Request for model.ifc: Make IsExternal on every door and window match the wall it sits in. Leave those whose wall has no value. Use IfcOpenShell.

First a look at what the model holds.

```python
import ifcopenshell
import ifcopenshell.util.element

model = ifcopenshell.open("model.ifc")
print(model.schema)
seen = {}
for e in model.by_type("IfcDoor") + model.by_type("IfcWindow"):
    if not e.FillsVoids:
        continue
    host = e.FillsVoids[0].RelatingOpeningElement.VoidsElements[0].RelatingBuildingElement
    own = ifcopenshell.util.element.get_pset(e, f"Pset_{e.is_a()[3:].removesuffix('StandardCase')}Common", "IsExternal")
    wall = ifcopenshell.util.element.get_pset(host, "Pset_WallCommon", "IsExternal")
    seen[e.is_a(), own, wall] = seen.get((e.is_a(), own, wall), 0) + 1
for (cls, own, wall), count in sorted(seen.items(), key=str):
    print(count, cls, "IsExternal:", own, "| host wall:", wall)
```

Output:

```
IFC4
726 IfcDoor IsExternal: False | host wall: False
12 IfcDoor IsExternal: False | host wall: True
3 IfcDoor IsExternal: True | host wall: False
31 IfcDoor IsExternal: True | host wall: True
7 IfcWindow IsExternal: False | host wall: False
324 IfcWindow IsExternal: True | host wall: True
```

```python
import ifcopenshell
import ifcopenshell.api.pset
import ifcopenshell.util.element

model = ifcopenshell.open("model.ifc")

count = 0
for ifc_class, pset_name in (("IfcDoor", "Pset_DoorCommon"), ("IfcWindow", "Pset_WindowCommon")):
    for e in model.by_type(ifc_class):
        if not e.FillsVoids:
            continue
        host = e.FillsVoids[0].RelatingOpeningElement.VoidsElements[0].RelatingBuildingElement
        external = ifcopenshell.util.element.get_pset(host, "Pset_WallCommon", "IsExternal")
        if external is None or ifcopenshell.util.element.get_pset(e, pset_name, "IsExternal") == external:
            continue
        pset = ifcopenshell.api.pset.add_pset(model, product=e, name=pset_name)
        ifcopenshell.api.pset.edit_pset(model, pset=pset, properties={"IsExternal": external})
        count += 1

print(count, "updated")

model.write("model-out.ifc")
```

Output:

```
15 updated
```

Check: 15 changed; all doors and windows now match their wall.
